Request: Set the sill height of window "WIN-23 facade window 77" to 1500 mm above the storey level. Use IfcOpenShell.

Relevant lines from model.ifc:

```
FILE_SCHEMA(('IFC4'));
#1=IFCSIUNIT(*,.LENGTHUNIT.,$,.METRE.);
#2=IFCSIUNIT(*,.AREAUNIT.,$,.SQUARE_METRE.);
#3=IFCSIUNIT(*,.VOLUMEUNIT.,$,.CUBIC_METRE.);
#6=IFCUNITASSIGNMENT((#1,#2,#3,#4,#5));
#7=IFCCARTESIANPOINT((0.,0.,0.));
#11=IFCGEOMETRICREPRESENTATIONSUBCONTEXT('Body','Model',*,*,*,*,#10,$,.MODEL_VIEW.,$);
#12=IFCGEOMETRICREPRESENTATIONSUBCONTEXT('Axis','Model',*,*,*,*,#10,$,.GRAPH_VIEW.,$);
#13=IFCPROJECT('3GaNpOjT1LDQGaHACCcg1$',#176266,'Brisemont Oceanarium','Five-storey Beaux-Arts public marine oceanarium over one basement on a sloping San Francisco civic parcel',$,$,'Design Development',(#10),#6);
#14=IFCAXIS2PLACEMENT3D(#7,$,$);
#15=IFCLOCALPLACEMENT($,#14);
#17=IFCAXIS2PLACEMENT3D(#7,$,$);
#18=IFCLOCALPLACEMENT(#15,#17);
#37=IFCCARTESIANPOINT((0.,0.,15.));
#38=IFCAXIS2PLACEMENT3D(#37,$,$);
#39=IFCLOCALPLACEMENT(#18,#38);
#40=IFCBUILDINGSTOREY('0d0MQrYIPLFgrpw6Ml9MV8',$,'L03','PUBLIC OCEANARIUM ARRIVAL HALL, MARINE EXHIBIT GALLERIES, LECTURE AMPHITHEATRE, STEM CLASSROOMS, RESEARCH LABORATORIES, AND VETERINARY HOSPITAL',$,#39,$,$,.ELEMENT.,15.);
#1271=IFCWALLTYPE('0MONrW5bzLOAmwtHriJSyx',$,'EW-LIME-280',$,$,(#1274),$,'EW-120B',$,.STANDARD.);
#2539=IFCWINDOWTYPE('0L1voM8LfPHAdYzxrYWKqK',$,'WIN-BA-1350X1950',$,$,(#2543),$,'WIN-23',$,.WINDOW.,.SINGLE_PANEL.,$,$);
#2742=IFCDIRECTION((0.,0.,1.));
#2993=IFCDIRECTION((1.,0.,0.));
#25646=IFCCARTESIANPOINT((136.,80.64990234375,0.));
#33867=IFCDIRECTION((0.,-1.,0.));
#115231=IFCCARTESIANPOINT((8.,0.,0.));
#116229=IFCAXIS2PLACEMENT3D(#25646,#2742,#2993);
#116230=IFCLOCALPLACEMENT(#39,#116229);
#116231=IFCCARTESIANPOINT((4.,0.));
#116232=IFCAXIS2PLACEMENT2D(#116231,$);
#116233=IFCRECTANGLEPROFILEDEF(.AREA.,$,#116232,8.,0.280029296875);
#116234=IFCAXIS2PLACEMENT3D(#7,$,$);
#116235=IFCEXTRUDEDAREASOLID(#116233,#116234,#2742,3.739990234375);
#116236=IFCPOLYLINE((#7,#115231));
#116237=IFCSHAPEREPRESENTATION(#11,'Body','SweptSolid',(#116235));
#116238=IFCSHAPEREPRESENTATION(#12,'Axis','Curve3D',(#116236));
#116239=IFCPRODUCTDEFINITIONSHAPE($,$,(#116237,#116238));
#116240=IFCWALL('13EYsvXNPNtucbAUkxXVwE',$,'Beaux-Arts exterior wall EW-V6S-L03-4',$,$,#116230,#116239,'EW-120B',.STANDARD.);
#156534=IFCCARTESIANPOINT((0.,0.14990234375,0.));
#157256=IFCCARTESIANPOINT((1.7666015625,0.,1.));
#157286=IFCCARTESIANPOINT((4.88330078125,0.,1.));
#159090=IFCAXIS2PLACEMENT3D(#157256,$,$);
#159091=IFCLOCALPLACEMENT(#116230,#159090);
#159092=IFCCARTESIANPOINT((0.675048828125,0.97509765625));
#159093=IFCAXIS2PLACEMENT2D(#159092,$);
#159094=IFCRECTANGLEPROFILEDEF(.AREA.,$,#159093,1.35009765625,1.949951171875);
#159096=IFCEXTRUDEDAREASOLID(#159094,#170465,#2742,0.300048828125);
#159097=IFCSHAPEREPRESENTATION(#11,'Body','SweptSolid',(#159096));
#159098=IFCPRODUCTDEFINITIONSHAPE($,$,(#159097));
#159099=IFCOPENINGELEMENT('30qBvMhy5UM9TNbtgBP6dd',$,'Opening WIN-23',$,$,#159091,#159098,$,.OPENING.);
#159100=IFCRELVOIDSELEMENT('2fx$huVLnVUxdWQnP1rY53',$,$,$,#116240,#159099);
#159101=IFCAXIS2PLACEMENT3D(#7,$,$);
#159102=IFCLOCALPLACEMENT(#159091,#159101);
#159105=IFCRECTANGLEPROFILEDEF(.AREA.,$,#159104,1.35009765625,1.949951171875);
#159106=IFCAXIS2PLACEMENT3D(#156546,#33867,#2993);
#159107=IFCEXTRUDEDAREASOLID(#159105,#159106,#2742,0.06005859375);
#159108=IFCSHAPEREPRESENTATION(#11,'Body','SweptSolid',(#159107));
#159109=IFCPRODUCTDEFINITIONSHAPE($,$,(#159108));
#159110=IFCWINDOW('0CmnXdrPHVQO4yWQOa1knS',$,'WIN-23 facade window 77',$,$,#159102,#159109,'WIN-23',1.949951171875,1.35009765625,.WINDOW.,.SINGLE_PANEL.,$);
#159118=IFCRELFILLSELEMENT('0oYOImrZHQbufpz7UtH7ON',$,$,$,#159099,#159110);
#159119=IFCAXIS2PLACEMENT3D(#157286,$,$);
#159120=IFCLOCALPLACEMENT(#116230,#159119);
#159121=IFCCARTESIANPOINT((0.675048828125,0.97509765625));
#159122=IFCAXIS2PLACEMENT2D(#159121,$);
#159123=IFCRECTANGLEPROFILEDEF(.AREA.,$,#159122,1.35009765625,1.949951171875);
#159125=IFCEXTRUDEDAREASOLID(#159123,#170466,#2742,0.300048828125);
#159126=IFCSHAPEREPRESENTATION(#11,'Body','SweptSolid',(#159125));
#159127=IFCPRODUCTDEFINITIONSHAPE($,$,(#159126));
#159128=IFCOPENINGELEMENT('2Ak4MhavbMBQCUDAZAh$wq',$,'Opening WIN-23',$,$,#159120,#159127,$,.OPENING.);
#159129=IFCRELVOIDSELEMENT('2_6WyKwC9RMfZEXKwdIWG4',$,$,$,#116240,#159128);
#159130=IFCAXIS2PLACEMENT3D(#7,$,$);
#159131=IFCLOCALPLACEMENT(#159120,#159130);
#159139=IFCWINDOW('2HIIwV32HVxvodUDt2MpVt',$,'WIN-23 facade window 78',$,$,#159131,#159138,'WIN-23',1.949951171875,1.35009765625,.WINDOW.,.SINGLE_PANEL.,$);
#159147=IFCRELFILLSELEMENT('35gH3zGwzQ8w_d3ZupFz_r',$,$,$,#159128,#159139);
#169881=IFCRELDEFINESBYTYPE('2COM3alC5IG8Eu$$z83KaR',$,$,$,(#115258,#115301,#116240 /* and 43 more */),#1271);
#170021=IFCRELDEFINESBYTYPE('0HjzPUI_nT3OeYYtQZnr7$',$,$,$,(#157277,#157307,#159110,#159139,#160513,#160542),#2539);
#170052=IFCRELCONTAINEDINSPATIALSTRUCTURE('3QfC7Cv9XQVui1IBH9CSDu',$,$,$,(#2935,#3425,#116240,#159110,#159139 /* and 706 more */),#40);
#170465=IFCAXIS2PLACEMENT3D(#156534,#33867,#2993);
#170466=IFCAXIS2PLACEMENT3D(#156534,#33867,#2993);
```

```python
import numpy as np
import ifcopenshell
import ifcopenshell.api.geometry
import ifcopenshell.geom
import ifcopenshell.util.element
import ifcopenshell.util.placement
import ifcopenshell.util.shape
import ifcopenshell.util.unit

model = ifcopenshell.open("model.ifc")
unit_scale = ifcopenshell.util.unit.calculate_unit_scale(model)

window = model.by_guid("0CmnXdrPHVQO4yWQOa1knS")
opening = window.FillsVoids[0].RelatingOpeningElement
storey = ifcopenshell.util.element.get_container(window, ifc_class="IfcBuildingStorey")
level = ifcopenshell.util.placement.get_local_placement(storey.ObjectPlacement)[2, 3]

# The opening's origin need not be at the sill, so measure its lowest point.
shape = ifcopenshell.geom.create_shape(ifcopenshell.geom.settings(), opening)
bottom = ifcopenshell.util.shape.get_shape_bottom_elevation(shape, shape.geometry) / unit_scale
dz = level + 1.5 / unit_scale - bottom

shift = np.array([0.0, 0.0, dz])
# The window is placed relative to its opening, so it follows when the opening moves.
matrix = ifcopenshell.util.placement.get_local_placement(opening.ObjectPlacement)
matrix[:3, 3] += shift
ifcopenshell.api.geometry.edit_object_placement(
    model, product=opening, matrix=matrix, is_si=False, should_transform_children=True
)

print(f"moved by {dz * unit_scale:+.3f} m")

model.write("model_v2.ifc")
```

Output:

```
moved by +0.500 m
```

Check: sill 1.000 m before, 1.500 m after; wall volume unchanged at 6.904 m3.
